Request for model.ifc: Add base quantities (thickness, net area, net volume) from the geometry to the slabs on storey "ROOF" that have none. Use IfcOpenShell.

First a look at what the model holds.

```python
import ifcopenshell
import ifcopenshell.util.element
import ifcopenshell.util.unit

model = ifcopenshell.open("model.ifc")
print(model.schema)
for unit_type in ("LENGTHUNIT", "AREAUNIT", "VOLUMEUNIT"):
    print(unit_type, ifcopenshell.util.unit.calculate_unit_scale(model, unit_type))
storey = next(s for s in model.by_type("IfcBuildingStorey") if s.Name == "ROOF")
slabs = [e for e in ifcopenshell.util.element.get_decomposition(storey) if e.is_a("IfcSlab")]
for e in sorted(slabs, key=lambda e: e.id()):
    print(e.id(), e.is_a(), e.Name, list(ifcopenshell.util.element.get_psets(e, qtos_only=True)), sep=" | ")
```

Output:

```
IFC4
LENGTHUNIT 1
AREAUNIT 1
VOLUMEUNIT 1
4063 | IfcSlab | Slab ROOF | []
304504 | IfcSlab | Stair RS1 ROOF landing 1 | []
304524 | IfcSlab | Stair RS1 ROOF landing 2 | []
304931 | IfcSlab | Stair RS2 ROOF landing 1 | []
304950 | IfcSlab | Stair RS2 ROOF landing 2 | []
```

```python
import ifcopenshell
import ifcopenshell.api.pset
import ifcopenshell.geom
import ifcopenshell.util.element
import ifcopenshell.util.shape
import ifcopenshell.util.unit

model = ifcopenshell.open("model.ifc")
unit_scale = ifcopenshell.util.unit.calculate_unit_scale(model)
area_scale = ifcopenshell.util.unit.calculate_unit_scale(model, "AREAUNIT")
volume_scale = ifcopenshell.util.unit.calculate_unit_scale(model, "VOLUMEUNIT")
settings = ifcopenshell.geom.settings()

storey = next(s for s in model.by_type("IfcBuildingStorey") if s.Name == "ROOF")
slabs = [e for e in ifcopenshell.util.element.get_decomposition(storey) if e.is_a("IfcSlab")]

for e in sorted(slabs, key=lambda e: e.id()):
    if ifcopenshell.util.element.get_psets(e, qtos_only=True, should_inherit=False):
        continue
    # Geometry comes back in metres, in the element's own axes.
    shape = ifcopenshell.geom.create_shape(settings, e)
    values = {
        "Width": ifcopenshell.util.shape.get_z(shape.geometry) / unit_scale,
        "NetArea": ifcopenshell.util.shape.get_footprint_area(shape.geometry) / area_scale,
        "NetVolume": ifcopenshell.util.shape.get_volume(shape.geometry) / volume_scale,
    }
    qto = ifcopenshell.api.pset.add_qto(model, product=e, name="Qto_SlabBaseQuantities")
    ifcopenshell.api.pset.edit_qto(model, qto=qto, properties=values)
    print(e.id(), {k: round(v, 3) for k, v in values.items()})

model.write("model_v2.ifc")
```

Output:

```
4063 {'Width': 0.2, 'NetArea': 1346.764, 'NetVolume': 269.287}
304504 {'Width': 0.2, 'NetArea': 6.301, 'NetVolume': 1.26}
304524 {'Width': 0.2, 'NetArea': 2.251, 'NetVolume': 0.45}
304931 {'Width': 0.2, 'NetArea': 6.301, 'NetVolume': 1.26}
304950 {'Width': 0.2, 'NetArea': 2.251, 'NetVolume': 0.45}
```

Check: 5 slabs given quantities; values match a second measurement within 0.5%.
